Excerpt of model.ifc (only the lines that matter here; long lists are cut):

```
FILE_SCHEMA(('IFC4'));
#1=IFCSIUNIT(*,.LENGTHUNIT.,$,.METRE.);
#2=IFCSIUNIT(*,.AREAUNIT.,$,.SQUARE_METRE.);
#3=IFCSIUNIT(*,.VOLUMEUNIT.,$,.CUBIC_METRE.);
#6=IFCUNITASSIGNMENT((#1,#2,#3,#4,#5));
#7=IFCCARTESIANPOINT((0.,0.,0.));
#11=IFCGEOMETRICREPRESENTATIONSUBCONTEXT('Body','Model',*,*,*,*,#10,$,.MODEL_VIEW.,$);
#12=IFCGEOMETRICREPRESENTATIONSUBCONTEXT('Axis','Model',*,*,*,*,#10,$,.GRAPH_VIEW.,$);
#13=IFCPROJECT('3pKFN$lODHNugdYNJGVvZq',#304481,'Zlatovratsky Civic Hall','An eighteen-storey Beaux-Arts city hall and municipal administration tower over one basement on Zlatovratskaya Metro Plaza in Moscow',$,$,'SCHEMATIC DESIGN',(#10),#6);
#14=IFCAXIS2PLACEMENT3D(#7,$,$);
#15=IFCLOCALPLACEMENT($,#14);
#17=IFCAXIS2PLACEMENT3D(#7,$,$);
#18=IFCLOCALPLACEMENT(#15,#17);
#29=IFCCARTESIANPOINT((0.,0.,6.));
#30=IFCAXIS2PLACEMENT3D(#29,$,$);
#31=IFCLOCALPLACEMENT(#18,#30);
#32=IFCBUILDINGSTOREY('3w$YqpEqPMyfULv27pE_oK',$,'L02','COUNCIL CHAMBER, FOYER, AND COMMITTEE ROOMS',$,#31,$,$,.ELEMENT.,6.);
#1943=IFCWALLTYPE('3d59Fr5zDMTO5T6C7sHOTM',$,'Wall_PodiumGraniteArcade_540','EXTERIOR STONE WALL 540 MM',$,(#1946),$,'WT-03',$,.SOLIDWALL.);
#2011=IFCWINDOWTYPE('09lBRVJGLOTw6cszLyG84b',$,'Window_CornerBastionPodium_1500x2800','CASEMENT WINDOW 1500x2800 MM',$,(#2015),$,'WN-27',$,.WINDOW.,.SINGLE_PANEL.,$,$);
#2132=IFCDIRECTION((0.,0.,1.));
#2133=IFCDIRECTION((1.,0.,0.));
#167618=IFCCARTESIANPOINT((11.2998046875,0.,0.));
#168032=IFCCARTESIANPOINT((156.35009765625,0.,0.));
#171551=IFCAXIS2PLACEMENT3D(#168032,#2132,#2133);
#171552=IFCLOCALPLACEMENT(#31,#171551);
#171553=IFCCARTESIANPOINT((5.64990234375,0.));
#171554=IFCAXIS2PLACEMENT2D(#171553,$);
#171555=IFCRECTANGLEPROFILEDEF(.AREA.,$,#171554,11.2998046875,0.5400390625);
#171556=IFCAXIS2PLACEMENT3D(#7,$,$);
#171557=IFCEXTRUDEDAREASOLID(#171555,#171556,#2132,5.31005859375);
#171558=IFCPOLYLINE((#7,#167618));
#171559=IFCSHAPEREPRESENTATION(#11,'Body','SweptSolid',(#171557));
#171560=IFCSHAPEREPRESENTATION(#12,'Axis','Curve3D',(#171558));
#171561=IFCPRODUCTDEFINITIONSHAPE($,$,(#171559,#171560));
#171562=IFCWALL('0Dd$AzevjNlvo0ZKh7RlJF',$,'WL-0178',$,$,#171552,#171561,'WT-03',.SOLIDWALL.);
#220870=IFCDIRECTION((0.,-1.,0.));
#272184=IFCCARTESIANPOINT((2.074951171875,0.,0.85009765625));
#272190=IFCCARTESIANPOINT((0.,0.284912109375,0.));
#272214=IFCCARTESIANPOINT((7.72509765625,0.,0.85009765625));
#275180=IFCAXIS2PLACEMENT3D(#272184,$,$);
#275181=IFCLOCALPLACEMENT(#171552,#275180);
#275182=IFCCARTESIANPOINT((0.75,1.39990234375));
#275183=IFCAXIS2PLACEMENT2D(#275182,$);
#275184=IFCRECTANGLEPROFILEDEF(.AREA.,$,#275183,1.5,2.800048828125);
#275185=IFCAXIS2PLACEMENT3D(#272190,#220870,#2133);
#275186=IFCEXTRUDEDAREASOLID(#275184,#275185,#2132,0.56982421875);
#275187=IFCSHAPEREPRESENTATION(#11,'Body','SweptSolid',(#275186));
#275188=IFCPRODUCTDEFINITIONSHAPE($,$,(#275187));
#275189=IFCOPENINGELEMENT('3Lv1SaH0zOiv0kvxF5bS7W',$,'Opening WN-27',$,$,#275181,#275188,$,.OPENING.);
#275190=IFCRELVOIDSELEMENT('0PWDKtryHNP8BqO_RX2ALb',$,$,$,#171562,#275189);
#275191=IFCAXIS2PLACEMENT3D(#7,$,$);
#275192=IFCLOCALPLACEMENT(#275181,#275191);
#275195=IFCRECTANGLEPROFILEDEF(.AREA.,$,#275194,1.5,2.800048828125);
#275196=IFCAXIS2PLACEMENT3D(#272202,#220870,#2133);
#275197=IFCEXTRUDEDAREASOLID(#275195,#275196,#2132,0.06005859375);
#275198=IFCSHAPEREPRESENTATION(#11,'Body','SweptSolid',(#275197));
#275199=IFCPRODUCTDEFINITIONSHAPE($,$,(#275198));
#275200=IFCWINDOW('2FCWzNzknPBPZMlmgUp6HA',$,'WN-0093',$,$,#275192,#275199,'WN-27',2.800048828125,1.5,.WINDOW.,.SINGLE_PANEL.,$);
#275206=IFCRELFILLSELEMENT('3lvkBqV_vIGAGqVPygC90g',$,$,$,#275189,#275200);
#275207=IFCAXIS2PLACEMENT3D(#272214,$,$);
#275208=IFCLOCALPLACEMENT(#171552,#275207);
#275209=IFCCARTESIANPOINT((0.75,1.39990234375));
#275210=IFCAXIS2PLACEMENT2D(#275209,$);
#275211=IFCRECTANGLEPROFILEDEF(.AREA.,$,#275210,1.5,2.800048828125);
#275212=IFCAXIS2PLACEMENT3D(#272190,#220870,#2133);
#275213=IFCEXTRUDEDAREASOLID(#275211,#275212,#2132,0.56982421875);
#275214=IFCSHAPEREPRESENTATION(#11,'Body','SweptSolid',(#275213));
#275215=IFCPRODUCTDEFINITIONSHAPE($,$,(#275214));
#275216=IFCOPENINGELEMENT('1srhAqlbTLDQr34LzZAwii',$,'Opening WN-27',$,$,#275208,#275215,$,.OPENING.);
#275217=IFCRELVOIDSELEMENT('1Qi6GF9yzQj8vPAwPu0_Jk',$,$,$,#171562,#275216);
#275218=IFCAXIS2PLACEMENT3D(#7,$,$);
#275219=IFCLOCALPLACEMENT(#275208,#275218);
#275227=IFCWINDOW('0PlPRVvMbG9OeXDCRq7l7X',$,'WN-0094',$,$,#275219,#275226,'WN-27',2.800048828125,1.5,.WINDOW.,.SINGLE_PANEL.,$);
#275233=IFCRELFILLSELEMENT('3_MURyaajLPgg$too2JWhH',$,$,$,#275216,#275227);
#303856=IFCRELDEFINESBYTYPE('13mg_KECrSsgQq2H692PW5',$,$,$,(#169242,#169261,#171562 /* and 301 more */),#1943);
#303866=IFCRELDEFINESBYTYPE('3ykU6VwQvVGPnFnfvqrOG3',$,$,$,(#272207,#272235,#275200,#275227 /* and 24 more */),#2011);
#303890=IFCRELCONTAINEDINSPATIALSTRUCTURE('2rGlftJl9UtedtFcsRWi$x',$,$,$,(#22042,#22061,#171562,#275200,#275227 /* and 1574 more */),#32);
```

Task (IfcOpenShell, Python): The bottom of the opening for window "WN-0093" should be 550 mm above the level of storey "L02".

```python
import numpy as np
import ifcopenshell
import ifcopenshell.api.geometry
import ifcopenshell.geom
import ifcopenshell.util.element
import ifcopenshell.util.placement
import ifcopenshell.util.shape
import ifcopenshell.util.unit

model = ifcopenshell.open("model.ifc")
unit_scale = ifcopenshell.util.unit.calculate_unit_scale(model)

window = model.by_guid("2FCWzNzknPBPZMlmgUp6HA")
opening = window.FillsVoids[0].RelatingOpeningElement
storey = ifcopenshell.util.element.get_container(window, ifc_class="IfcBuildingStorey")
level = ifcopenshell.util.placement.get_local_placement(storey.ObjectPlacement)[2, 3]

# The opening's origin need not be at the sill, so measure its lowest point.
shape = ifcopenshell.geom.create_shape(ifcopenshell.geom.settings(), opening)
bottom = ifcopenshell.util.shape.get_shape_bottom_elevation(shape, shape.geometry) / unit_scale
dz = level + 0.55 - bottom

shift = np.array([0.0, 0.0, dz])
# The window is placed relative to its opening, so it follows when the opening moves.
matrix = ifcopenshell.util.placement.get_local_placement(opening.ObjectPlacement)
matrix[:3, 3] += shift
ifcopenshell.api.geometry.edit_object_placement(
    model, product=opening, matrix=matrix, is_si=False, should_transform_children=True
)

print(f"moved by {dz * unit_scale:+.3f} m")

model.write("model_v2.ifc")
```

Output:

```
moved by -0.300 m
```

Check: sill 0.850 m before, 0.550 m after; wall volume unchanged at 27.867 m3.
